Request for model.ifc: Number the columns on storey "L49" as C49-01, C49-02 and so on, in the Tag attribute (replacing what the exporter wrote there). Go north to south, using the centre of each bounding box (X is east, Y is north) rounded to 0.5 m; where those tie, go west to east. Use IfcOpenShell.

First a look at what the model holds.

```python
import ifcopenshell
import ifcopenshell.util.element
import ifcopenshell.util.placement

model = ifcopenshell.open("model.ifc")
print(model.schema)
storey = next(s for s in model.by_type("IfcBuildingStorey") if s.Name == "L49")
columns = [e for e in ifcopenshell.util.element.get_decomposition(storey) if e.is_a("IfcColumn")]
for e in sorted(columns, key=lambda e: e.id()):
    origin = ifcopenshell.util.placement.get_local_placement(e.ObjectPlacement)[:3, 3]
    print(e.id(), e.Tag, e.Name, origin.round(2) + 0.0, sep=" | ")
```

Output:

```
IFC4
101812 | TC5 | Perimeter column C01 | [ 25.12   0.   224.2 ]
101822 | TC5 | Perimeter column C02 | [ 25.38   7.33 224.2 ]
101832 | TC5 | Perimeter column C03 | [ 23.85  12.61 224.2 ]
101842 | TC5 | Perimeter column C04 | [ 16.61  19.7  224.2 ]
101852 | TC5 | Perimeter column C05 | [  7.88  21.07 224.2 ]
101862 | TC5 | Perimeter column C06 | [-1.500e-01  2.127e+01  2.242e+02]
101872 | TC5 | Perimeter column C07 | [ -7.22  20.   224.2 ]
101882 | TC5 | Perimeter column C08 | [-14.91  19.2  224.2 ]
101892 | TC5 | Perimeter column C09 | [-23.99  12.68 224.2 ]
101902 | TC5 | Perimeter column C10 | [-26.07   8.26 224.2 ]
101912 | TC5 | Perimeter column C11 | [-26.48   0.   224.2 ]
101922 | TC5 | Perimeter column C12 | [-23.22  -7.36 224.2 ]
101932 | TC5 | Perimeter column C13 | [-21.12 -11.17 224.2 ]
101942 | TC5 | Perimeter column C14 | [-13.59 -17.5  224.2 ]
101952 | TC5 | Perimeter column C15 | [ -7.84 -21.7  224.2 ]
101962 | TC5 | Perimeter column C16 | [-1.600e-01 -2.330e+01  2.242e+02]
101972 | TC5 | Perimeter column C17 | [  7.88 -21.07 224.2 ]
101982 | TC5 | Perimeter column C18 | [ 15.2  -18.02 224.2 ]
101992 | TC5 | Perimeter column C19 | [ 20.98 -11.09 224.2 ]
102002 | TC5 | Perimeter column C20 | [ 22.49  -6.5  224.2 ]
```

```python
import ifcopenshell
import ifcopenshell.geom
import ifcopenshell.util.element
import ifcopenshell.util.shape

model = ifcopenshell.open("model.ifc")
settings = ifcopenshell.geom.settings()
settings.set("use-world-coords", True)


def centre(element):
    shape = ifcopenshell.geom.create_shape(settings, element)
    return ifcopenshell.util.shape.get_bbox_centroid(shape.geometry)


storey = next(s for s in model.by_type("IfcBuildingStorey") if s.Name == "L49")
columns = [e for e in ifcopenshell.util.element.get_decomposition(storey) if e.is_a("IfcColumn")]

# Insertion points can sit at a corner or the storey origin, so sort by the geometry (in metres).
centres = {e: centre(e) for e in columns}
columns.sort(key=lambda e: (-round(centres[e][1] / 0.5), centres[e][0]))

for i, e in enumerate(columns, start=1):
    number = f"C49-{i:02d}"
    e.Tag = number
    print(e.id(), number)

model.write("model_v2.ifc")
```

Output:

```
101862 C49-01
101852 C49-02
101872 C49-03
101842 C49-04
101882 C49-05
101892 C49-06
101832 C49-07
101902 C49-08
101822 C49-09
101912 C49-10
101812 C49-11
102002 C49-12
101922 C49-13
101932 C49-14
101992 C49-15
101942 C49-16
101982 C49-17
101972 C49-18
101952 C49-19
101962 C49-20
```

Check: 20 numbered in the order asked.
